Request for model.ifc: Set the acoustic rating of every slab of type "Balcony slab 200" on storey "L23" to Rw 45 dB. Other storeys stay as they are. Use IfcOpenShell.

First a look at what the model holds.

```python
import ifcopenshell
import ifcopenshell.util.element

model = ifcopenshell.open("model.ifc")
print(model.schema)
storey = next(s for s in model.by_type("IfcBuildingStorey") if s.Name == "L23")
slabs = [e for e in ifcopenshell.util.element.get_decomposition(storey) if e.is_a("IfcSlab")]
seen = {}
for e in slabs:
    element_type = ifcopenshell.util.element.get_type(e)
    key = (element_type.Name if element_type != e and element_type else None, ifcopenshell.util.element.get_pset(e, "Pset_SlabCommon", "AcousticRating"))
    seen[key] = seen.get(key, 0) + 1
for (name, value), count in sorted(seen.items(), key=str):
    print(count, "x", name, "|", value)
```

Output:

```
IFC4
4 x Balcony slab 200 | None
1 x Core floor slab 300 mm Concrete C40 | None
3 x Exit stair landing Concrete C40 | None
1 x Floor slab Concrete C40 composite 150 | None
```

```python
import ifcopenshell
import ifcopenshell.api.pset
import ifcopenshell.util.element

model = ifcopenshell.open("model.ifc")

storey = next(s for s in model.by_type("IfcBuildingStorey") if s.Name == "L23")
slabs = [e for e in ifcopenshell.util.element.get_decomposition(storey) if e.is_a("IfcSlab")]

count = 0
for e in slabs:
    element_type = ifcopenshell.util.element.get_type(e)
    if element_type in (None, e) or element_type.Name != "Balcony slab 200":
        continue
    found = ifcopenshell.util.element.get_pset(e, "Pset_SlabCommon", should_inherit=False)
    if found:
        pset = model.by_id(found["id"])
        if len(ifcopenshell.util.element.get_elements_by_pset(pset)) > 1:
            pset = ifcopenshell.api.pset.unshare_pset(model, products=[e], pset=pset)[0]
    else:
        pset = ifcopenshell.api.pset.add_pset(model, product=e, name="Pset_SlabCommon")
    ifcopenshell.api.pset.edit_pset(model, pset=pset, properties={"AcousticRating": "Rw 45 dB"})
    count += 1

print(count, "slabs updated")

model.write("model-out.ifc")
```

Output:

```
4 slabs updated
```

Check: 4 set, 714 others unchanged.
